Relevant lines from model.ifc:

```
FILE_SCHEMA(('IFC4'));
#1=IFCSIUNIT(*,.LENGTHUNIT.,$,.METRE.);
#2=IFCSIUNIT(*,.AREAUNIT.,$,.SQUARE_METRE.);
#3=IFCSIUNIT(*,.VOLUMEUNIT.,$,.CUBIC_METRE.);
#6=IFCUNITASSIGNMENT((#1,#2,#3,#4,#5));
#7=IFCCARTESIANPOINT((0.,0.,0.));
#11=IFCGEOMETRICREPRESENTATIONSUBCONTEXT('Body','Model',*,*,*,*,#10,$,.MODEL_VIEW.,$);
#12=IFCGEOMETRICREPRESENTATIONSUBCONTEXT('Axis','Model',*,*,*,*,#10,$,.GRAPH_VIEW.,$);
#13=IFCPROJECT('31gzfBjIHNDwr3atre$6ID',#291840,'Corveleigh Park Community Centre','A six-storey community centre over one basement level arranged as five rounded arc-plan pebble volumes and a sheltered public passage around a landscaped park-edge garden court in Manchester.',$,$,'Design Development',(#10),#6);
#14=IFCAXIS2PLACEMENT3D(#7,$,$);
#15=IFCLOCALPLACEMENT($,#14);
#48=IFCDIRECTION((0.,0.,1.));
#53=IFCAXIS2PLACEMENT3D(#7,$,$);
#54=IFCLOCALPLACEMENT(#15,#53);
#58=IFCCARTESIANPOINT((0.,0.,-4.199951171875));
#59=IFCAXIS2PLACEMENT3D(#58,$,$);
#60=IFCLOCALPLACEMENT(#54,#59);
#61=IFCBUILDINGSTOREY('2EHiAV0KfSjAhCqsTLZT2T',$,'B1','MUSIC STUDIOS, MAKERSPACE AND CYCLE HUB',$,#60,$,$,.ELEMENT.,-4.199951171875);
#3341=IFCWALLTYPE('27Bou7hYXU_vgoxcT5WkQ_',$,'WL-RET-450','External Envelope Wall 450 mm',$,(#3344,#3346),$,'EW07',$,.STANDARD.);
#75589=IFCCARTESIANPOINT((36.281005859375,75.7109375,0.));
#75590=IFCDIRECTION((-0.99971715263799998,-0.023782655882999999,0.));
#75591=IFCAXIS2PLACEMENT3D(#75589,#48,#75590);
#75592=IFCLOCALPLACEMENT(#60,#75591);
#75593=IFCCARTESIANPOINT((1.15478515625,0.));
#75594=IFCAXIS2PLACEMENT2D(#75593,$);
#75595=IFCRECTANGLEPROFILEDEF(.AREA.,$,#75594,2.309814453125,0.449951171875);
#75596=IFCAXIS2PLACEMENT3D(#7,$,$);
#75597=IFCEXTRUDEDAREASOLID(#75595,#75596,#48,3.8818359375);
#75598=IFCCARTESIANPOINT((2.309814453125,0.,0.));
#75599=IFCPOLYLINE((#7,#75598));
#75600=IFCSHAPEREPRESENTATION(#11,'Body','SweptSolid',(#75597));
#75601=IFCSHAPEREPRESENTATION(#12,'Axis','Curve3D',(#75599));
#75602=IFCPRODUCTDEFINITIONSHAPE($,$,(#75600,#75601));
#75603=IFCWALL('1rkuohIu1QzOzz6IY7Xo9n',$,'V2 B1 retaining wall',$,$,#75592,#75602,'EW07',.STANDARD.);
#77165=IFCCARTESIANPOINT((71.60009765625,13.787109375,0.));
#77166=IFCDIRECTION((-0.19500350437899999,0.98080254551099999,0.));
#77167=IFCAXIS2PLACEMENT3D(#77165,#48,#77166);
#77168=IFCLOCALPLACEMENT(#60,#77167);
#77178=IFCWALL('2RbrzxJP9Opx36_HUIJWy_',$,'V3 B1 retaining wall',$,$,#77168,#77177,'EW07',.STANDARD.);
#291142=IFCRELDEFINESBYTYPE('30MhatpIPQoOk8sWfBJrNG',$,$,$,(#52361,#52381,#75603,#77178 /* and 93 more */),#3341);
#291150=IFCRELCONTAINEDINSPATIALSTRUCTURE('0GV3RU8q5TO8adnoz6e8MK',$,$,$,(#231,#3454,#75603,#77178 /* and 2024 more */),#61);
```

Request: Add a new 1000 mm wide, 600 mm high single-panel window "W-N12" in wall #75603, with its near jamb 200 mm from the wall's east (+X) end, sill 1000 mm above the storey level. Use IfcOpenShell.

```python
import numpy as np
import ifcopenshell
import ifcopenshell.api.feature
import ifcopenshell.api.geometry
import ifcopenshell.api.root
import ifcopenshell.api.spatial
import ifcopenshell.geom
import ifcopenshell.util.element
import ifcopenshell.util.placement
import ifcopenshell.util.representation
import ifcopenshell.util.shape
import ifcopenshell.util.unit

model = ifcopenshell.open("model.ifc")
unit_scale = ifcopenshell.util.unit.calculate_unit_scale(model)
settings = ifcopenshell.geom.settings()


def volume(element):
    """Net volume in cubic metres, openings subtracted."""
    shape = ifcopenshell.geom.create_shape(settings, element)
    return ifcopenshell.util.shape.get_volume(shape.geometry)


wall = model.by_guid("1rkuohIu1QzOzz6IY7Xo9n")
storey = ifcopenshell.util.element.get_container(wall, ifc_class="IfcBuildingStorey")
context = ifcopenshell.util.representation.get_context(model, "Model", "Body", "MODEL_VIEW")
before = volume(wall)

width, height, from_end, sill = 1, 0.6, 0.2, 1  # metres

# The wall runs along its own X axis, and the end named is its -X end.
wall_shape = ifcopenshell.geom.create_shape(settings, wall)
x, y, z = ifcopenshell.util.shape.get_vertices(wall_shape.geometry).T
start = x.min() + from_end
face, thickness = float(y.min()), float(y.max() - y.min())
wall_matrix = ifcopenshell.util.placement.get_local_placement(wall.ObjectPlacement)
level = ifcopenshell.util.placement.get_local_placement(storey.ObjectPlacement)[2, 3]


def in_wall(x, y):
    """Placement at x, y metres in the wall's axes, at sill height."""
    matrix = wall_matrix.copy()
    matrix[:, 3] = wall_matrix @ np.array([x / unit_scale, y / unit_scale, 0.0, 1.0])
    matrix[2, 3] = level + sill / unit_scale
    return matrix


# Opening: a box that overshoots both wall faces by 50 mm.
opening = ifcopenshell.api.root.create_entity(model, ifc_class="IfcOpeningElement", predefined_type="OPENING")
box = ifcopenshell.api.geometry.add_wall_representation(
    model, context=context, length=width, height=height, thickness=thickness + 0.1
)
ifcopenshell.api.geometry.assign_representation(model, product=opening, representation=box)
ifcopenshell.api.geometry.edit_object_placement(model, product=opening, matrix=in_wall(start, face - 0.05), is_si=False)
ifcopenshell.api.feature.add_feature(model, feature=opening, element=wall)

window = ifcopenshell.api.root.create_entity(model, ifc_class="IfcWindow", name="W-N12", predefined_type="WINDOW")
window.OverallWidth, window.OverallHeight = width / unit_scale, height / unit_scale
window.PartitioningType = "SINGLE_PANEL"
body = ifcopenshell.api.geometry.add_window_representation(
    model,
    context=context,
    overall_width=window.OverallWidth,
    overall_height=window.OverallHeight,
    partition_type="SINGLE_PANEL",
)
ifcopenshell.api.geometry.assign_representation(model, product=window, representation=body)
ifcopenshell.api.spatial.assign_container(model, products=[window], relating_structure=storey)
ifcopenshell.api.feature.add_filling(model, opening=opening, element=window)

# Centre the window in the wall's thickness.
ifcopenshell.api.geometry.edit_object_placement(model, product=window, matrix=in_wall(start, face), is_si=False)
window_shape = ifcopenshell.geom.create_shape(settings, window)
depth = ifcopenshell.util.shape.get_vertices(window_shape.geometry)[:, 1]
offset = face + thickness / 2 - (depth.min() + depth.max()) / 2
ifcopenshell.api.geometry.edit_object_placement(model, product=window, matrix=in_wall(start, offset), is_si=False)

after = volume(wall)

print(f"wall volume {before:.3f} -> {after:.3f} m3")

model.write("model_v2.ifc")
```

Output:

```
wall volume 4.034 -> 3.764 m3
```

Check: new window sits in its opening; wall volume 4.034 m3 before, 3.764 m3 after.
